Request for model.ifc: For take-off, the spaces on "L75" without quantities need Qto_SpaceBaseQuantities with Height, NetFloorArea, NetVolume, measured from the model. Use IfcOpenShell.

First a look at what the model holds.

```python
import ifcopenshell
import ifcopenshell.util.element
import ifcopenshell.util.unit

model = ifcopenshell.open("model.ifc")
print(model.schema)
for unit_type in ("LENGTHUNIT", "AREAUNIT", "VOLUMEUNIT"):
    print(unit_type, ifcopenshell.util.unit.calculate_unit_scale(model, unit_type))
storey = next(s for s in model.by_type("IfcBuildingStorey") if s.Name == "L75")
spaces = [e for e in ifcopenshell.util.element.get_decomposition(storey) if e.is_a("IfcSpace")]
for e in sorted(spaces, key=lambda e: e.id()):
    print(e.id(), e.is_a(), e.Name, list(ifcopenshell.util.element.get_psets(e, qtos_only=True)), sep=" | ")
```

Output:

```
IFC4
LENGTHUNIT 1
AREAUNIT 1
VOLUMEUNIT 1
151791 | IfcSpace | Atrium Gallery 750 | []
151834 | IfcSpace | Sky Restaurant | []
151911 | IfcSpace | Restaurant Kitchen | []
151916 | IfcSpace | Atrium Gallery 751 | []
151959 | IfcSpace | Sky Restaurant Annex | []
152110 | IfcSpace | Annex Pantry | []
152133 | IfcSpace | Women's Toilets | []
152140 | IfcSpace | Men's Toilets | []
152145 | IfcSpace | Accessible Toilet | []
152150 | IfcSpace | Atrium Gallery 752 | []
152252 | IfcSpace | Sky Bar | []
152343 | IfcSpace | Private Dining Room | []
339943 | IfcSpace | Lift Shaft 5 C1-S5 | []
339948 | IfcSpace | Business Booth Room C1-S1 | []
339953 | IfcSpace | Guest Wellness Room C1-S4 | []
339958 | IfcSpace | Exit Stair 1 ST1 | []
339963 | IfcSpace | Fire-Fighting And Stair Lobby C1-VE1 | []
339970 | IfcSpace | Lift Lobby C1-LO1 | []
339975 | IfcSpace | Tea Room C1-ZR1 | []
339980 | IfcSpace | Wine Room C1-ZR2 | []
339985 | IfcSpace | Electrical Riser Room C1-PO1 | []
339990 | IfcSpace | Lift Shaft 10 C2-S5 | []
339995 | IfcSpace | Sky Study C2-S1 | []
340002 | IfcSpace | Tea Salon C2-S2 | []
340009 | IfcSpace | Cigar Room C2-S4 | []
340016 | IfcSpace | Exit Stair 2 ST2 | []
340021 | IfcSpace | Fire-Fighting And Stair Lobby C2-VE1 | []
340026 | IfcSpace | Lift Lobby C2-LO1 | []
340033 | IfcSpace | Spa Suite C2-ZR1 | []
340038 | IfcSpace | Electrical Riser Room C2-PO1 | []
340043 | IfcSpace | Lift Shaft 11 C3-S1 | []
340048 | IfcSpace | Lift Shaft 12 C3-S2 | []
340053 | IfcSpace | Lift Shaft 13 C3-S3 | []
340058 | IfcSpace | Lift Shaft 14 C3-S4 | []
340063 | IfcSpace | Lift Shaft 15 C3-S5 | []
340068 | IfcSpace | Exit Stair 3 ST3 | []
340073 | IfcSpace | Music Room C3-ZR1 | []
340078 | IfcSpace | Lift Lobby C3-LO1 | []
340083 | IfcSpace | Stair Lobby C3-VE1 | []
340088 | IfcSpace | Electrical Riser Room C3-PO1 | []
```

```python
import ifcopenshell
import ifcopenshell.api.pset
import ifcopenshell.geom
import ifcopenshell.util.element
import ifcopenshell.util.shape
import ifcopenshell.util.unit

model = ifcopenshell.open("model.ifc")
unit_scale = ifcopenshell.util.unit.calculate_unit_scale(model)
area_scale = ifcopenshell.util.unit.calculate_unit_scale(model, "AREAUNIT")
volume_scale = ifcopenshell.util.unit.calculate_unit_scale(model, "VOLUMEUNIT")
settings = ifcopenshell.geom.settings()

storey = next(s for s in model.by_type("IfcBuildingStorey") if s.Name == "L75")
spaces = [e for e in ifcopenshell.util.element.get_decomposition(storey) if e.is_a("IfcSpace")]

for e in sorted(spaces, key=lambda e: e.id()):
    if ifcopenshell.util.element.get_psets(e, qtos_only=True, should_inherit=False):
        continue
    # Geometry comes back in metres, in the element's own axes.
    shape = ifcopenshell.geom.create_shape(settings, e)
    values = {
        "Height": ifcopenshell.util.shape.get_z(shape.geometry) / unit_scale,
        "NetFloorArea": ifcopenshell.util.shape.get_footprint_area(shape.geometry) / area_scale,
        "NetVolume": ifcopenshell.util.shape.get_volume(shape.geometry) / volume_scale,
    }
    qto = ifcopenshell.api.pset.add_qto(model, product=e, name="Qto_SpaceBaseQuantities")
    ifcopenshell.api.pset.edit_qto(model, qto=qto, properties=values)
    print(e.id(), {k: round(v, 3) for k, v in values.items()})

model.write("model_rev.ifc")
```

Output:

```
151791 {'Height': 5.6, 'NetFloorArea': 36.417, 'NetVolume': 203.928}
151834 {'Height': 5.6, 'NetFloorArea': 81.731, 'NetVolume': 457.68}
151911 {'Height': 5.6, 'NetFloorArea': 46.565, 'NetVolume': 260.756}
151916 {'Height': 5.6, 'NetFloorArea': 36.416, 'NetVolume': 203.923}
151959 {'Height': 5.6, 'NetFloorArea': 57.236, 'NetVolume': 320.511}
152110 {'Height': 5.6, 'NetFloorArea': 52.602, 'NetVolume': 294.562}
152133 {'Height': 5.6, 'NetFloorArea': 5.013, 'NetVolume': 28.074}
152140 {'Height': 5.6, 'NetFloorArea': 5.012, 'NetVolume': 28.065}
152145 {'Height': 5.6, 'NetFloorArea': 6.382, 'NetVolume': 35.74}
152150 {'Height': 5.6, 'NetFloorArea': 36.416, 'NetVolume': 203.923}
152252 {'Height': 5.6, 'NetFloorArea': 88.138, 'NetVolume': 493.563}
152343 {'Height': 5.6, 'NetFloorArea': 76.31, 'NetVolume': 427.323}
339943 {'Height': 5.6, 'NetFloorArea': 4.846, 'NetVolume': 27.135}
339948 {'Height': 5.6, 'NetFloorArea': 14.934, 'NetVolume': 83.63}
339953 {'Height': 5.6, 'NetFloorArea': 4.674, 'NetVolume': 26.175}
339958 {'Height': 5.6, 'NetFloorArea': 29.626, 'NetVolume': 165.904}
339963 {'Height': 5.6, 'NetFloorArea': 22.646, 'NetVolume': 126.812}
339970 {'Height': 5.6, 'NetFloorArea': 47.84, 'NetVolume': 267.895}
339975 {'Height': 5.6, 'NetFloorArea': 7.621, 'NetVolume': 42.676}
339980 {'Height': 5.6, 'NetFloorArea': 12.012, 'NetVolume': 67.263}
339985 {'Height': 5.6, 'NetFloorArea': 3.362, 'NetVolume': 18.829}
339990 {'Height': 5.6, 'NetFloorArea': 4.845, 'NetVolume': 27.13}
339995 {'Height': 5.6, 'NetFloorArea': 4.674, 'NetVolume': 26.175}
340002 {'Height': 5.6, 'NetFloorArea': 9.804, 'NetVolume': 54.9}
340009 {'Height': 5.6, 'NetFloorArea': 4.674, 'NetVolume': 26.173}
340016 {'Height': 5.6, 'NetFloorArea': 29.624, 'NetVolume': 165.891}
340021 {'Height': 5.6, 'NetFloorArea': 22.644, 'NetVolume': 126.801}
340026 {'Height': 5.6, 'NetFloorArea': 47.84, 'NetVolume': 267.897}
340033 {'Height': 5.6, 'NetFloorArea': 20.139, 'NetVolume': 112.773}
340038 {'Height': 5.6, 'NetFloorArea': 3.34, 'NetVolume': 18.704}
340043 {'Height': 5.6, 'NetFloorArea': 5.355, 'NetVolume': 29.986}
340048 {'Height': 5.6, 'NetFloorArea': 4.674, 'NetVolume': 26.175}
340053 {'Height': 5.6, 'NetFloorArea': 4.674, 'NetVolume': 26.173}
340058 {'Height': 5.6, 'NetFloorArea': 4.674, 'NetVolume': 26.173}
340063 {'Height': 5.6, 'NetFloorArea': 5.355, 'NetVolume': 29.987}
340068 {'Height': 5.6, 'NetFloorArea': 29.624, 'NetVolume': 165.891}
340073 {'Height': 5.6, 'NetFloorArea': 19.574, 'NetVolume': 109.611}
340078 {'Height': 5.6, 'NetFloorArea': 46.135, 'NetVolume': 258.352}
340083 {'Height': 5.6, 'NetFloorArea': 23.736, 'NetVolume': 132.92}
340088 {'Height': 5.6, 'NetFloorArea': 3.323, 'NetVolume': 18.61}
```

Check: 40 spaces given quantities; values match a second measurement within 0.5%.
